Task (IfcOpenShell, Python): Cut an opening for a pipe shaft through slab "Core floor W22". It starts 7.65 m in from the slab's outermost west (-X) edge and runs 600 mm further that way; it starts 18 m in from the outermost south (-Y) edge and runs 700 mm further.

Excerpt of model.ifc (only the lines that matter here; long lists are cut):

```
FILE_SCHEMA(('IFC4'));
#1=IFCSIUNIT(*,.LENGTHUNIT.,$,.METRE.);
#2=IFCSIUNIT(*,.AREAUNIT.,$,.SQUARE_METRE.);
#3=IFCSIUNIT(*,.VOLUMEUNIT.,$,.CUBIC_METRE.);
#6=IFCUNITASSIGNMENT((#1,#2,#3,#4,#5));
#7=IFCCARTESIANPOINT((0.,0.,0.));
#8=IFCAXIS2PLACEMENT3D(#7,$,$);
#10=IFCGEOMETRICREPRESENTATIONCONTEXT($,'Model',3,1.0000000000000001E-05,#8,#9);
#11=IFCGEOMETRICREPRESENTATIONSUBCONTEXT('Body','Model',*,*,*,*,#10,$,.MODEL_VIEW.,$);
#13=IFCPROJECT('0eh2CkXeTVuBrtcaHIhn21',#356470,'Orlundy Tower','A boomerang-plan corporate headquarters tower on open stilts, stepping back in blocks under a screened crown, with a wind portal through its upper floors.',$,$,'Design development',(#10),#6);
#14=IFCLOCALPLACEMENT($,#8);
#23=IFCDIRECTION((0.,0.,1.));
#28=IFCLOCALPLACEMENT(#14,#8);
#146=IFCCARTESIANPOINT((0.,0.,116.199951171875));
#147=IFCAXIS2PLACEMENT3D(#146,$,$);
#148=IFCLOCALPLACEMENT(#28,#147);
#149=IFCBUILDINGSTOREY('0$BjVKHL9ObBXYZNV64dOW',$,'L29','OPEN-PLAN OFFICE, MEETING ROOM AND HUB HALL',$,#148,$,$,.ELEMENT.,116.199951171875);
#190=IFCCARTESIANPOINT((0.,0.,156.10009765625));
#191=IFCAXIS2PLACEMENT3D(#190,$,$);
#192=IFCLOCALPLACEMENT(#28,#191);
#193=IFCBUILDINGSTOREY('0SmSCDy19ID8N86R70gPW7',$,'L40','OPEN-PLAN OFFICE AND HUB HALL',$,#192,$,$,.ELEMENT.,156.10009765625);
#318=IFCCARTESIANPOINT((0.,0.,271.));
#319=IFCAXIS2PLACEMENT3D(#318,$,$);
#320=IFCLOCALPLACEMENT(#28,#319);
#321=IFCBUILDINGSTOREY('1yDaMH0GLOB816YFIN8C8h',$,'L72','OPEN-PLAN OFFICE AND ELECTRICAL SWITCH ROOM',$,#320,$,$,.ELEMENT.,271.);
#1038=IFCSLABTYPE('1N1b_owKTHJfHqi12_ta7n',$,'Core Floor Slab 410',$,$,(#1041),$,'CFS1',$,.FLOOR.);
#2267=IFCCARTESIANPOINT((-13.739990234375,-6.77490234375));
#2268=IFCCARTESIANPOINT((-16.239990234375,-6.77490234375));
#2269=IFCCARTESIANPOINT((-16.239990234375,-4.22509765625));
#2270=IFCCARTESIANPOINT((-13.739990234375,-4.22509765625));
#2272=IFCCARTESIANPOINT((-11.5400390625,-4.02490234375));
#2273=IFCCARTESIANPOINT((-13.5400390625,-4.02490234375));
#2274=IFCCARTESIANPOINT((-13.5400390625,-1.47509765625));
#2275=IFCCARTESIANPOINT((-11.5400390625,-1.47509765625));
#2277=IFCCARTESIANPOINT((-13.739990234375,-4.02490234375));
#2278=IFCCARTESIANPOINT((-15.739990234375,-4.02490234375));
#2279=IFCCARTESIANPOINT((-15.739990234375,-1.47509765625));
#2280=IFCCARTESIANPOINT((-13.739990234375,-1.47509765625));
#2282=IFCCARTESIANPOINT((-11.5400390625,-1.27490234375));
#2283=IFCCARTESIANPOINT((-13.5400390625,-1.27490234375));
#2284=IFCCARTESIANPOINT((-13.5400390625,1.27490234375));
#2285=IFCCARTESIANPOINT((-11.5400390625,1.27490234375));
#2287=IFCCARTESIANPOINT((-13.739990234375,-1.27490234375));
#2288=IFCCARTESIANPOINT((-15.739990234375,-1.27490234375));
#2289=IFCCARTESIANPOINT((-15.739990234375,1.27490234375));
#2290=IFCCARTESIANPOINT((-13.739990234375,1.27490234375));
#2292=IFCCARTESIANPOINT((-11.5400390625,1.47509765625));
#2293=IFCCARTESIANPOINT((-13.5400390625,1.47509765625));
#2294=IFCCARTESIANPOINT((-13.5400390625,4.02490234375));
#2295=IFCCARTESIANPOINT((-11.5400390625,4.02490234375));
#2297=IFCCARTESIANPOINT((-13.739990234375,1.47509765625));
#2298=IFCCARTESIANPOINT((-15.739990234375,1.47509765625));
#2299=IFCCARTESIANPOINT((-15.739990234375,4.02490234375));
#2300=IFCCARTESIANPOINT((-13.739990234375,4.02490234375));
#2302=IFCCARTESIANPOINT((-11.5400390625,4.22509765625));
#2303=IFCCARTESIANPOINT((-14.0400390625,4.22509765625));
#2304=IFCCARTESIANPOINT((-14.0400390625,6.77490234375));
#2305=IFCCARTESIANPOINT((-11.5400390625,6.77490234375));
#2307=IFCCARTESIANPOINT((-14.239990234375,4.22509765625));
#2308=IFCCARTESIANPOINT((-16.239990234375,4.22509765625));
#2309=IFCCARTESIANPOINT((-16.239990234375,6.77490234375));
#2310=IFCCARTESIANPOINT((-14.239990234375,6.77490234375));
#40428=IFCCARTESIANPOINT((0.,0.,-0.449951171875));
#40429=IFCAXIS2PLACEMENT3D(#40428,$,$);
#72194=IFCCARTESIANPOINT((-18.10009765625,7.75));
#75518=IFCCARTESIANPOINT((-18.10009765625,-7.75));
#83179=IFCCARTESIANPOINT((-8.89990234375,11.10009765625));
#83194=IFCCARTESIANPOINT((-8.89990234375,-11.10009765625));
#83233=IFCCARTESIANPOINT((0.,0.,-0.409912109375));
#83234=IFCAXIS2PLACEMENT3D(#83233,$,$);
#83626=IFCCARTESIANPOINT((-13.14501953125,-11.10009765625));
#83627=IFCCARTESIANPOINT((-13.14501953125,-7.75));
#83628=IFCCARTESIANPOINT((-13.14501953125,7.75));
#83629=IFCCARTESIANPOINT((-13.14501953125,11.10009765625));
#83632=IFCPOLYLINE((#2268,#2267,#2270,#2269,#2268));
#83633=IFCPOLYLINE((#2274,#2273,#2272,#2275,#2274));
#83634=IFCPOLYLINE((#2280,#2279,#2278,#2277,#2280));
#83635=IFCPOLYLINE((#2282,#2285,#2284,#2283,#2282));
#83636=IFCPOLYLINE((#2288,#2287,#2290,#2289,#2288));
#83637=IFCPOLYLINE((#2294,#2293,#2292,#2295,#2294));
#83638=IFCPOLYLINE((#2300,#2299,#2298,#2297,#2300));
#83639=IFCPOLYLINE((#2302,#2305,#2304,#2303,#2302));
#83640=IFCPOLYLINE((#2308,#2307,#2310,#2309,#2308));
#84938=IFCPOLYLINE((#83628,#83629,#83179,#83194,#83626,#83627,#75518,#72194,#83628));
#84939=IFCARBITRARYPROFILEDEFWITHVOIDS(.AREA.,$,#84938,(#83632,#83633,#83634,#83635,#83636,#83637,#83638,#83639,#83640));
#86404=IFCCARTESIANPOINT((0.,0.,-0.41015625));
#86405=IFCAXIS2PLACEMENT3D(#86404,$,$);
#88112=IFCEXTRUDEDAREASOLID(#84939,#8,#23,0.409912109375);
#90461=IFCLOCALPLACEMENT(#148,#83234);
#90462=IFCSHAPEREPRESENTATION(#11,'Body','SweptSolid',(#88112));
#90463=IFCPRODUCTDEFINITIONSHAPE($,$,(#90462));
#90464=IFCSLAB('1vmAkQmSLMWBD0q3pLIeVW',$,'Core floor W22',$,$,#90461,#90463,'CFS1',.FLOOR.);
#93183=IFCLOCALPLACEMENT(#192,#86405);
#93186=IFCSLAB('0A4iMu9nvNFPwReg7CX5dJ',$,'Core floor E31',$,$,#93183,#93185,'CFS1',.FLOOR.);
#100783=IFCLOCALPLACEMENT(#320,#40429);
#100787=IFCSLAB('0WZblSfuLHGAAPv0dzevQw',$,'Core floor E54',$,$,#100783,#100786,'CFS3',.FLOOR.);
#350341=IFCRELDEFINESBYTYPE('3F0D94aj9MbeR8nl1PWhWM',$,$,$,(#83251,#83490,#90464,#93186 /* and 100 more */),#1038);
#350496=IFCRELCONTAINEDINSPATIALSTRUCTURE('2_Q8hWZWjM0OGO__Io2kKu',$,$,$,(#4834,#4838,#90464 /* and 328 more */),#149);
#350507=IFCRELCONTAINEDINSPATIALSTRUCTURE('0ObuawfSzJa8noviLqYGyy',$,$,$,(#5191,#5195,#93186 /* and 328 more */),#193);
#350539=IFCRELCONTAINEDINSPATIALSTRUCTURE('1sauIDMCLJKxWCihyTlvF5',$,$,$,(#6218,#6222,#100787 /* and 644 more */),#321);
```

```python
import numpy as np
import ifcopenshell
import ifcopenshell.api.feature
import ifcopenshell.api.geometry
import ifcopenshell.api.root
import ifcopenshell.geom
import ifcopenshell.util.placement
import ifcopenshell.util.representation
import ifcopenshell.util.shape
import ifcopenshell.util.unit

model = ifcopenshell.open("model.ifc")
unit_scale = ifcopenshell.util.unit.calculate_unit_scale(model)
settings = ifcopenshell.geom.settings()


def volume(element):
    """Net volume in cubic metres, openings subtracted."""
    shape = ifcopenshell.geom.create_shape(settings, element)
    return ifcopenshell.util.shape.get_volume(shape.geometry)


slab = model.by_id(90464)
before = volume(slab)

# Extent in the slab's own axes, in metres. The edges named are its -X and -Y sides.
slab_shape = ifcopenshell.geom.create_shape(settings, slab)
vertices = ifcopenshell.util.shape.get_vertices(slab_shape.geometry)
x_min, y_min, bottom = vertices.min(axis=0)
top = vertices[:, 2].max()

opening = ifcopenshell.api.root.create_entity(model, ifc_class="IfcOpeningElement", name="Pipe shaft opening", predefined_type="OPENING")
context = ifcopenshell.util.representation.get_context(model, "Model", "Body", "MODEL_VIEW")
width, depth = 0.6, 0.7
outline = [(0.0, 0.0), (width, 0.0), (width, depth), (0.0, depth), (0.0, 0.0)]
# Overshoot both faces by 50 mm so the cut is clean.
shape = ifcopenshell.api.geometry.add_slab_representation(
    model, context=context, depth=top - bottom + 0.1, polyline=outline
)
ifcopenshell.api.geometry.assign_representation(model, product=opening, representation=shape)

matrix = ifcopenshell.util.placement.get_local_placement(slab.ObjectPlacement)
matrix[:, 3] = matrix @ np.append(np.array([x_min + 7.65, y_min + 18, bottom - 0.05]) / unit_scale, 1.0)
ifcopenshell.api.geometry.edit_object_placement(model, product=opening, matrix=matrix, is_si=False)
ifcopenshell.api.feature.add_feature(model, feature=opening, element=slab)

after = volume(slab)

print(f"slab volume {before:.3f} -> {after:.3f} m3")

model.write("model_v2.ifc")
```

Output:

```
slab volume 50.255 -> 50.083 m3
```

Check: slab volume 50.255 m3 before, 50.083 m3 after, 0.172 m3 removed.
